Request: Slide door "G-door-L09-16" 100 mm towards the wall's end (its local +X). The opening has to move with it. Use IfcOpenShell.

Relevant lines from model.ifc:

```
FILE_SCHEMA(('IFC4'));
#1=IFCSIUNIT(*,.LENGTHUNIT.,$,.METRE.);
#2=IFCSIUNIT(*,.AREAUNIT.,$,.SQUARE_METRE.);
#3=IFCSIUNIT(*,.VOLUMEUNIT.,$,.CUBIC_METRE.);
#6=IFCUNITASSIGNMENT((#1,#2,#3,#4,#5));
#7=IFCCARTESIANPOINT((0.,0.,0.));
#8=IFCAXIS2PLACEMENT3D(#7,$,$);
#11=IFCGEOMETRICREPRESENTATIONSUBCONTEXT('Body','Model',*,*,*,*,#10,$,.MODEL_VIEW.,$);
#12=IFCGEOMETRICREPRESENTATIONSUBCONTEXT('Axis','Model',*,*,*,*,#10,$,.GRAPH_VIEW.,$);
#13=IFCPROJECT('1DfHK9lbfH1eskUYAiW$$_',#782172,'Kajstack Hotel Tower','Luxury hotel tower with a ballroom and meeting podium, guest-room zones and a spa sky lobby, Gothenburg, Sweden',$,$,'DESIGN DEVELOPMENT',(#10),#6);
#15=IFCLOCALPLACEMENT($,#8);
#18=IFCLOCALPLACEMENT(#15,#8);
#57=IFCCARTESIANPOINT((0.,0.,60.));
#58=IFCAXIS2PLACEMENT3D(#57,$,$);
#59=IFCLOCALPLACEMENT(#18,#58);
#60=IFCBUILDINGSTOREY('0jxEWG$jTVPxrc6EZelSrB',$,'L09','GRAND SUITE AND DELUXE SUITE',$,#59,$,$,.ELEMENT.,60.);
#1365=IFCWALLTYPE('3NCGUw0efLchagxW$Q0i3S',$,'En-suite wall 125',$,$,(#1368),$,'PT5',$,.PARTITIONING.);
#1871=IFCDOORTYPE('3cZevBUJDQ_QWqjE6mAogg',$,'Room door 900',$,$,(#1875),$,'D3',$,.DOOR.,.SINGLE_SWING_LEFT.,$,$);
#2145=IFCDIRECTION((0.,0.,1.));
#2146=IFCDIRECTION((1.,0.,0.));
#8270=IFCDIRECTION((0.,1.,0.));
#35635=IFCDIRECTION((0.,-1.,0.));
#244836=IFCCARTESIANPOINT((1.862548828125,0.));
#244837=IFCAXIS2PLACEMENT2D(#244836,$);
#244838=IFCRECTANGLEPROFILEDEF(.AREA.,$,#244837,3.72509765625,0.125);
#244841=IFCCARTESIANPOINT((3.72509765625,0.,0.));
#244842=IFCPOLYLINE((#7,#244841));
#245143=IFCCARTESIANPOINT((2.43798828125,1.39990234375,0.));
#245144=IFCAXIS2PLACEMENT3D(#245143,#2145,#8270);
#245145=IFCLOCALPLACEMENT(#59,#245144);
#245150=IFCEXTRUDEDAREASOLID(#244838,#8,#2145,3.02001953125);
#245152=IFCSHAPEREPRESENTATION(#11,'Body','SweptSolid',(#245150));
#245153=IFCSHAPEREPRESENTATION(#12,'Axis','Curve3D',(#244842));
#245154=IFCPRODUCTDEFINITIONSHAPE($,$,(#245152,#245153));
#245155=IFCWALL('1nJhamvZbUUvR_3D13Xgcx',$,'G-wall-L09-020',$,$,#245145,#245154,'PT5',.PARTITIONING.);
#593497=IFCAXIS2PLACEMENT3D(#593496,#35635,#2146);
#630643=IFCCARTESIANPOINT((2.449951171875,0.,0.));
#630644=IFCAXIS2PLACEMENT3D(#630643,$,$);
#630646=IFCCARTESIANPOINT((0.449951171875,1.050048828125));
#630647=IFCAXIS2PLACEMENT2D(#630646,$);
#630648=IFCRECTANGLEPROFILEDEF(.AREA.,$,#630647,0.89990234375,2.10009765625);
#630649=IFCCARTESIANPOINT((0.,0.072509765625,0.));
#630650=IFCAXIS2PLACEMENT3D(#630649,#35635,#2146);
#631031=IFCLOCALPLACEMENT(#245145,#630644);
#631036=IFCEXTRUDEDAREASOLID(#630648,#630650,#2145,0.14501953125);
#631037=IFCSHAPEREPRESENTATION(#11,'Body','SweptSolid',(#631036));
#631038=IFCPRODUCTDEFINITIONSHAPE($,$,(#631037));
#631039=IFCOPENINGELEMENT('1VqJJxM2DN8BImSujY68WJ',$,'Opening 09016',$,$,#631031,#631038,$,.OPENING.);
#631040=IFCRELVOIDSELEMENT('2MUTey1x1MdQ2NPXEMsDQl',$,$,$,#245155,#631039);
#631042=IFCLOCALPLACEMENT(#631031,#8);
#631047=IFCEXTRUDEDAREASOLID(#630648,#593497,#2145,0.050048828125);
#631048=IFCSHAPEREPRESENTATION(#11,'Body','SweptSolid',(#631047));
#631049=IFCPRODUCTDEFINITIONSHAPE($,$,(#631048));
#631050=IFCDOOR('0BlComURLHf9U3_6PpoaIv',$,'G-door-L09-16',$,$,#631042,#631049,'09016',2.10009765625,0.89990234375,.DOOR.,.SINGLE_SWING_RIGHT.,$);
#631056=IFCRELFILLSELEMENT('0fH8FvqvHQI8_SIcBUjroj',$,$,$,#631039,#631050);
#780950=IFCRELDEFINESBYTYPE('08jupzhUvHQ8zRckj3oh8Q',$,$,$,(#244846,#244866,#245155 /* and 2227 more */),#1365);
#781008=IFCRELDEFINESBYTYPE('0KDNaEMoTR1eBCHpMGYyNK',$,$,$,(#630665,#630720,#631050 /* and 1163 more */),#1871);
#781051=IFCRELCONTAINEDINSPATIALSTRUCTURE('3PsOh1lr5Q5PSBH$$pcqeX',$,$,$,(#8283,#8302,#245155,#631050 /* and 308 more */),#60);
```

```python
import ifcopenshell
import ifcopenshell.api.geometry
import ifcopenshell.util.placement
import ifcopenshell.util.unit

model = ifcopenshell.open("model.ifc")
unit_scale = ifcopenshell.util.unit.calculate_unit_scale(model)

door = model.by_id(631050)
opening = door.FillsVoids[0].RelatingOpeningElement
wall = opening.VoidsElements[0].RelatingBuildingElement

wall_matrix = ifcopenshell.util.placement.get_local_placement(wall.ObjectPlacement)
shift = wall_matrix[:3, 0] * 0.1 / unit_scale
before = ifcopenshell.util.placement.get_local_placement(door.ObjectPlacement)[:3, 3].copy()

# The door is placed relative to its opening, so it follows when the opening moves.
matrix = ifcopenshell.util.placement.get_local_placement(opening.ObjectPlacement)
matrix[:3, 3] += shift
ifcopenshell.api.geometry.edit_object_placement(
    model, product=opening, matrix=matrix, is_si=False, should_transform_children=True
)

after = ifcopenshell.util.placement.get_local_placement(door.ObjectPlacement)[:3, 3]
print("door moved by", (after - before).round(3) + 0.0)

model.write("model_v2.ifc")
```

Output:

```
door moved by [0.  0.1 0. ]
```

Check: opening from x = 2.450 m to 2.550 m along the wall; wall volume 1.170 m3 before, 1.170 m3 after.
